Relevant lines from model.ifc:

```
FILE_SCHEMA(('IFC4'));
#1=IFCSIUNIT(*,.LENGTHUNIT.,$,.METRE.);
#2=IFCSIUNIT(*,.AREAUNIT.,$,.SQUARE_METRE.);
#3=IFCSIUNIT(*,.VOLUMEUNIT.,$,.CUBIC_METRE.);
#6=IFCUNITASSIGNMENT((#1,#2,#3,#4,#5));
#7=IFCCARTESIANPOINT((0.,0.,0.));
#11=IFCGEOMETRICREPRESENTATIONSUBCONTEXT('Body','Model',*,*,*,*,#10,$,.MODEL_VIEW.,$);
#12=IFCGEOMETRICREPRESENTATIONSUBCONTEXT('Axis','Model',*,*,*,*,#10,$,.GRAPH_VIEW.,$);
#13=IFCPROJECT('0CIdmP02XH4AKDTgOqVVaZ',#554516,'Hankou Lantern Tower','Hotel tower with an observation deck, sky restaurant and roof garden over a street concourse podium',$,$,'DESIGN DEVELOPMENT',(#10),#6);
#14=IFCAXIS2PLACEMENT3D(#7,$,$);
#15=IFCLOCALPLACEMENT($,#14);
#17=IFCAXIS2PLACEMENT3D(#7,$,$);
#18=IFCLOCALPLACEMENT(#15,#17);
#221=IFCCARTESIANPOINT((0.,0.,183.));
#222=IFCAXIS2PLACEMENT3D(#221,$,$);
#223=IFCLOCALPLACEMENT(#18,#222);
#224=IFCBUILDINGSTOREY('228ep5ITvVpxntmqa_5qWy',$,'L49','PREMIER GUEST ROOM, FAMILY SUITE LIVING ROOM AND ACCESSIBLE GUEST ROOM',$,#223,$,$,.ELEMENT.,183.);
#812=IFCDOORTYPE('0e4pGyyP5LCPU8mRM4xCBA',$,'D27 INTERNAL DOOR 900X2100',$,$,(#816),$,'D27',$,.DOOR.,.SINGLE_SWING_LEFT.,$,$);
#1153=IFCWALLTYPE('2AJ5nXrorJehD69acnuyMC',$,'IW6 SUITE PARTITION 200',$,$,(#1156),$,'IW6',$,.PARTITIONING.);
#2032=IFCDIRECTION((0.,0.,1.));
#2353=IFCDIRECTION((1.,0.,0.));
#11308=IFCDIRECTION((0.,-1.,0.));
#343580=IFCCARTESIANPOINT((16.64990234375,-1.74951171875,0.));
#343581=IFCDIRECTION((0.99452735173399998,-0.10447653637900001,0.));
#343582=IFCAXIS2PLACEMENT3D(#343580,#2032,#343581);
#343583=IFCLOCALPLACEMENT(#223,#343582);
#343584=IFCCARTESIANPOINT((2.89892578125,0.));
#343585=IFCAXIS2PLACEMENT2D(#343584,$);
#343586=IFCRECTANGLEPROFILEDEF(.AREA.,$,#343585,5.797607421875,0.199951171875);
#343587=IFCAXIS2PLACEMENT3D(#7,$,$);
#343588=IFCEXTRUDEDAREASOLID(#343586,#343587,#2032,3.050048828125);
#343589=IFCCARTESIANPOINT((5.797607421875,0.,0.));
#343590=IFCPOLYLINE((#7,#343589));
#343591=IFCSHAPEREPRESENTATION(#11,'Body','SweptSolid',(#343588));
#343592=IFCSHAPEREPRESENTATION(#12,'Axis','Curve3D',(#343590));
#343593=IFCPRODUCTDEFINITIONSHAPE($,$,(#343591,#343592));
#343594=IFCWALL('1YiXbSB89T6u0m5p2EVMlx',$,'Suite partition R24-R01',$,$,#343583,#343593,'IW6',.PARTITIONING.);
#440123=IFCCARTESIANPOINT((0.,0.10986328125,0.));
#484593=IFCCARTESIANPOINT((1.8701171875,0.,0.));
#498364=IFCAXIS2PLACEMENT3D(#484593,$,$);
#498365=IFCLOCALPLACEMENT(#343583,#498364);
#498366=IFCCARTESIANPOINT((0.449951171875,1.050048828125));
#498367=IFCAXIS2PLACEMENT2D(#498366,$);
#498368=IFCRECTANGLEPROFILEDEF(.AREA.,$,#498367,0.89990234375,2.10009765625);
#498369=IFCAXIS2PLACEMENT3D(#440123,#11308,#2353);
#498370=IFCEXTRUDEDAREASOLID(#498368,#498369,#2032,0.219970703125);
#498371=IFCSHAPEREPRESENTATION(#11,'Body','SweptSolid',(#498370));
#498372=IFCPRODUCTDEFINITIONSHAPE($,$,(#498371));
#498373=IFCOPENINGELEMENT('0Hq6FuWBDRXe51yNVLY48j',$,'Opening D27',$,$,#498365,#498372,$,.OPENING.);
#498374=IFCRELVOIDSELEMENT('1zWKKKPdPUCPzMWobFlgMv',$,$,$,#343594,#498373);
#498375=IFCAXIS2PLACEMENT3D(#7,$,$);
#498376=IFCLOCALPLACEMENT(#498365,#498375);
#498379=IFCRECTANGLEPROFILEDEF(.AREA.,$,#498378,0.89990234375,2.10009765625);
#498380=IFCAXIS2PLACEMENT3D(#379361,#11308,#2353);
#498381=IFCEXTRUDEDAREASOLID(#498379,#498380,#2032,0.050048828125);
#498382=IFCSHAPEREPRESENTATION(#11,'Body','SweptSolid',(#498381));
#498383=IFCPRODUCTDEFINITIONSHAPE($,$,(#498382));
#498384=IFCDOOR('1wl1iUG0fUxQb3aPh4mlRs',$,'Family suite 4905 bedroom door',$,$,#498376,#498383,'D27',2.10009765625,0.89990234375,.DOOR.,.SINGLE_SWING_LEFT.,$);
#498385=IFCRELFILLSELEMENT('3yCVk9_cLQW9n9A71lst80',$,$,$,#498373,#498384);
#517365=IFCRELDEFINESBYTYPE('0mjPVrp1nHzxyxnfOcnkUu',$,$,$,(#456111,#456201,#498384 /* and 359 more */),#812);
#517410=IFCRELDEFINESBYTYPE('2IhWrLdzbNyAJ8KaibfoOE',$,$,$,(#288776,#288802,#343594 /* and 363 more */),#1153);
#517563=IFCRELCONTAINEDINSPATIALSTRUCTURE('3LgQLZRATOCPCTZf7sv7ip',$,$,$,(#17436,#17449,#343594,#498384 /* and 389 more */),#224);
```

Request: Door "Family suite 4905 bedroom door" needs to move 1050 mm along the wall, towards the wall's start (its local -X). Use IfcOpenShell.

```python
import ifcopenshell
import ifcopenshell.api.geometry
import ifcopenshell.util.placement

model = ifcopenshell.open("model.ifc")

door = model.by_id(498384)
opening = door.FillsVoids[0].RelatingOpeningElement
wall = opening.VoidsElements[0].RelatingBuildingElement

wall_matrix = ifcopenshell.util.placement.get_local_placement(wall.ObjectPlacement)
shift = wall_matrix[:3, 0] * -1.05
before = ifcopenshell.util.placement.get_local_placement(door.ObjectPlacement)[:3, 3].copy()

# The door is placed relative to its opening, so it follows when the opening moves.
matrix = ifcopenshell.util.placement.get_local_placement(opening.ObjectPlacement)
matrix[:3, 3] += shift
ifcopenshell.api.geometry.edit_object_placement(
    model, product=opening, matrix=matrix, is_si=False, should_transform_children=True
)

after = ifcopenshell.util.placement.get_local_placement(door.ObjectPlacement)[:3, 3]
print("door moved by", (after - before).round(3) + 0.0)

model.write("model_rev.ifc")
```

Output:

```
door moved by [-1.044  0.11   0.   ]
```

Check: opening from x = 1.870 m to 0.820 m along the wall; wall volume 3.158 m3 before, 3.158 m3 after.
